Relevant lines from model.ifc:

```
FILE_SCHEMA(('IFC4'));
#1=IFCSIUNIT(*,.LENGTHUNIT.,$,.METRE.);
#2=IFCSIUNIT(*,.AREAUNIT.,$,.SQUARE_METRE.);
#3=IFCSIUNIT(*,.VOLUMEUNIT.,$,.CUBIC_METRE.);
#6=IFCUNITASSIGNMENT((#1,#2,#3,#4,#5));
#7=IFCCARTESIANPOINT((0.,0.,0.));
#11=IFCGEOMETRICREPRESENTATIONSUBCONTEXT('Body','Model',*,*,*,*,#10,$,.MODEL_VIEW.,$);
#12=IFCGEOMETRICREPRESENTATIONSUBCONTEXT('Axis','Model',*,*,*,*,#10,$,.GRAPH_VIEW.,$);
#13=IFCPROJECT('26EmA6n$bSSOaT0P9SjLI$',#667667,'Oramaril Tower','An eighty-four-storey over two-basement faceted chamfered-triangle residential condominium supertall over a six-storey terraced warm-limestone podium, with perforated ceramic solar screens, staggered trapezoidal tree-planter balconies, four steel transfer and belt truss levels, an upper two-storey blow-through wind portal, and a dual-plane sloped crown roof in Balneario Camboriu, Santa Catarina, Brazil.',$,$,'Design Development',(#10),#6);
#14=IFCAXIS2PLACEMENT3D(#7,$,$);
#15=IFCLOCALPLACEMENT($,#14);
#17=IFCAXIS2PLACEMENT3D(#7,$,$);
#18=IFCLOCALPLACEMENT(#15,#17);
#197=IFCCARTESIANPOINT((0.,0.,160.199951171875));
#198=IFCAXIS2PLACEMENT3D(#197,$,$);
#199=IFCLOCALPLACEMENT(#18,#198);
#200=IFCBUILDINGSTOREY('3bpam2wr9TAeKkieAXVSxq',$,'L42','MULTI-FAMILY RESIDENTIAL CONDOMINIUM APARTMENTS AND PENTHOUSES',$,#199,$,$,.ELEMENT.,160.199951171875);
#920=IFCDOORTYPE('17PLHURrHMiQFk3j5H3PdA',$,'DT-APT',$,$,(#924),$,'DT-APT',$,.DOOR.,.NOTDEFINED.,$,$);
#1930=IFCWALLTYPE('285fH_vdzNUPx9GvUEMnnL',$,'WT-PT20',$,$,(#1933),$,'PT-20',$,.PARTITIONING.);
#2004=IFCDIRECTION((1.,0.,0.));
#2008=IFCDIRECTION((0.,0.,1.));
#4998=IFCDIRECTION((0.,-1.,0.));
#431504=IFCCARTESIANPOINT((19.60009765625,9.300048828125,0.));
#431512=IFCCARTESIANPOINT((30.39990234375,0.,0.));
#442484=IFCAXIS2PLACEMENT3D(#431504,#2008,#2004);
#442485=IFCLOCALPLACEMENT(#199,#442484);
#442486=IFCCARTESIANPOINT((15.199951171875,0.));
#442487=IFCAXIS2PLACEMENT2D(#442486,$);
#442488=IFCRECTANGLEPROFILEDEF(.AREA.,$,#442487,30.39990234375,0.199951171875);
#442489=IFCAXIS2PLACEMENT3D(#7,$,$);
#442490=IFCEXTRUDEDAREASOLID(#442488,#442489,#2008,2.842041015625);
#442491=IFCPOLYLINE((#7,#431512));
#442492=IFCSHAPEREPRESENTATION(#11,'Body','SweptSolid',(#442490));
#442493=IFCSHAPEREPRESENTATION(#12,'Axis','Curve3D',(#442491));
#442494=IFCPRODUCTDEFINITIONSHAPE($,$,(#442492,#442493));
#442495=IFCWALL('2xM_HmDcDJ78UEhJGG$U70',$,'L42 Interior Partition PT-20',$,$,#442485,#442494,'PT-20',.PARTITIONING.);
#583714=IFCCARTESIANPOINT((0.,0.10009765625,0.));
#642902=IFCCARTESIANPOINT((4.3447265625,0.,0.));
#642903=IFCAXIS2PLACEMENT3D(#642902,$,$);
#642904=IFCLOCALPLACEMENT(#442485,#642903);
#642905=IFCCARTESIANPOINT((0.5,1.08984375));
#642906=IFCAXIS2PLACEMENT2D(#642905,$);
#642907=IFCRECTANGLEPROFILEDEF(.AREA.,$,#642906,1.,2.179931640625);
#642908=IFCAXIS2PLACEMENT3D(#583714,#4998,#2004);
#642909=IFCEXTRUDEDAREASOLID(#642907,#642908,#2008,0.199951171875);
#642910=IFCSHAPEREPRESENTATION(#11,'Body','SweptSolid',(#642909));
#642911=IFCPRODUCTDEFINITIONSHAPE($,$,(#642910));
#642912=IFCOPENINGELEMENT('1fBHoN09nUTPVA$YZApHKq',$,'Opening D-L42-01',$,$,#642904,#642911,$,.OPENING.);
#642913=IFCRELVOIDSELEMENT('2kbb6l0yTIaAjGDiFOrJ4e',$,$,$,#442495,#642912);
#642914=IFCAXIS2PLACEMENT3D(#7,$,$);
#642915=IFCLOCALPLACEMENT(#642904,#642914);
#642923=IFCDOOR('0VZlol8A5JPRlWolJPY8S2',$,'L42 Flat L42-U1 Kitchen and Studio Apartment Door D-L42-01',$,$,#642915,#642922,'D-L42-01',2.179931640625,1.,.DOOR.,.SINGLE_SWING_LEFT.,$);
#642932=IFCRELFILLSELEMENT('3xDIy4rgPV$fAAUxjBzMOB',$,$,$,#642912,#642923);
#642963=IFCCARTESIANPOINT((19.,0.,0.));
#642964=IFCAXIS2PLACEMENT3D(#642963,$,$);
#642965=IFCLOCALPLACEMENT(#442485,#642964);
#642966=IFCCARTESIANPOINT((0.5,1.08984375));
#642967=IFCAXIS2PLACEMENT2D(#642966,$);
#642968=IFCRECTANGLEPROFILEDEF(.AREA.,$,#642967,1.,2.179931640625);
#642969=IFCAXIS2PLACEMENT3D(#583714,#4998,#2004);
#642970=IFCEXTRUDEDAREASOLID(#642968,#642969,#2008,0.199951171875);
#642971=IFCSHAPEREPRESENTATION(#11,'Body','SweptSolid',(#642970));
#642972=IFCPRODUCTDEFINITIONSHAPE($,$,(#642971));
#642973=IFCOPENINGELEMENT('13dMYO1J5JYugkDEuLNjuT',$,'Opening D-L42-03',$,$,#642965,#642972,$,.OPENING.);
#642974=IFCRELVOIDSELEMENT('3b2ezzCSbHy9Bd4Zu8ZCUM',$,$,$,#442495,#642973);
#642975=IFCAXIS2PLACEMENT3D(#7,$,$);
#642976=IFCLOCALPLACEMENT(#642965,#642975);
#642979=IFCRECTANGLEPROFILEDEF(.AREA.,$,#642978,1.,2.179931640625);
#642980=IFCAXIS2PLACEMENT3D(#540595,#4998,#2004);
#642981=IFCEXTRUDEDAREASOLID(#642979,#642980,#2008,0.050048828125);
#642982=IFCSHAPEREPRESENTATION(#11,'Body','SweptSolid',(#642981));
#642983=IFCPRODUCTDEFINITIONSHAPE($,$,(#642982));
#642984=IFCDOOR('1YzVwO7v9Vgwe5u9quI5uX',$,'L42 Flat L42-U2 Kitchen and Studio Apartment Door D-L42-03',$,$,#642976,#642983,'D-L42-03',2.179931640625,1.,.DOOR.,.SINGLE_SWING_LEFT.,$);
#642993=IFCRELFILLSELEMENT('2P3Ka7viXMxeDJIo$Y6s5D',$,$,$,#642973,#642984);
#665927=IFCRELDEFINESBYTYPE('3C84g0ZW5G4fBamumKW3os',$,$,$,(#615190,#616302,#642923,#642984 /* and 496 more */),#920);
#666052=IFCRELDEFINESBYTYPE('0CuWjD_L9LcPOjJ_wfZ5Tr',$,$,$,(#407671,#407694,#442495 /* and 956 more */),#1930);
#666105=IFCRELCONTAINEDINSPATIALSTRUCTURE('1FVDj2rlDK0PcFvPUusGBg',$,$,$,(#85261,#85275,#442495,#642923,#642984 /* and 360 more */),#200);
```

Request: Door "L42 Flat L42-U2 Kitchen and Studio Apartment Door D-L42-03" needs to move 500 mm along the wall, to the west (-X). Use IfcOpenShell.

```python
import ifcopenshell
import ifcopenshell.api.geometry
import ifcopenshell.util.placement
import ifcopenshell.util.unit

model = ifcopenshell.open("model.ifc")
unit_scale = ifcopenshell.util.unit.calculate_unit_scale(model)

door = model.by_guid("1YzVwO7v9Vgwe5u9quI5uX")
opening = door.FillsVoids[0].RelatingOpeningElement
wall = opening.VoidsElements[0].RelatingBuildingElement

wall_matrix = ifcopenshell.util.placement.get_local_placement(wall.ObjectPlacement)
shift = wall_matrix[:3, 0] * -0.5 / unit_scale
before = ifcopenshell.util.placement.get_local_placement(door.ObjectPlacement)[:3, 3].copy()

# The door is placed relative to its opening, so it follows when the opening moves.
matrix = ifcopenshell.util.placement.get_local_placement(opening.ObjectPlacement)
matrix[:3, 3] += shift
ifcopenshell.api.geometry.edit_object_placement(
    model, product=opening, matrix=matrix, is_si=False, should_transform_children=True
)

after = ifcopenshell.util.placement.get_local_placement(door.ObjectPlacement)[:3, 3]
print("door moved by", (after - before).round(3) + 0.0)

model.write("model_updated.ifc")
```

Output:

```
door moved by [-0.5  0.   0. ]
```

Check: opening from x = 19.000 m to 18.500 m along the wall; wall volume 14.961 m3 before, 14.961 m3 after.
